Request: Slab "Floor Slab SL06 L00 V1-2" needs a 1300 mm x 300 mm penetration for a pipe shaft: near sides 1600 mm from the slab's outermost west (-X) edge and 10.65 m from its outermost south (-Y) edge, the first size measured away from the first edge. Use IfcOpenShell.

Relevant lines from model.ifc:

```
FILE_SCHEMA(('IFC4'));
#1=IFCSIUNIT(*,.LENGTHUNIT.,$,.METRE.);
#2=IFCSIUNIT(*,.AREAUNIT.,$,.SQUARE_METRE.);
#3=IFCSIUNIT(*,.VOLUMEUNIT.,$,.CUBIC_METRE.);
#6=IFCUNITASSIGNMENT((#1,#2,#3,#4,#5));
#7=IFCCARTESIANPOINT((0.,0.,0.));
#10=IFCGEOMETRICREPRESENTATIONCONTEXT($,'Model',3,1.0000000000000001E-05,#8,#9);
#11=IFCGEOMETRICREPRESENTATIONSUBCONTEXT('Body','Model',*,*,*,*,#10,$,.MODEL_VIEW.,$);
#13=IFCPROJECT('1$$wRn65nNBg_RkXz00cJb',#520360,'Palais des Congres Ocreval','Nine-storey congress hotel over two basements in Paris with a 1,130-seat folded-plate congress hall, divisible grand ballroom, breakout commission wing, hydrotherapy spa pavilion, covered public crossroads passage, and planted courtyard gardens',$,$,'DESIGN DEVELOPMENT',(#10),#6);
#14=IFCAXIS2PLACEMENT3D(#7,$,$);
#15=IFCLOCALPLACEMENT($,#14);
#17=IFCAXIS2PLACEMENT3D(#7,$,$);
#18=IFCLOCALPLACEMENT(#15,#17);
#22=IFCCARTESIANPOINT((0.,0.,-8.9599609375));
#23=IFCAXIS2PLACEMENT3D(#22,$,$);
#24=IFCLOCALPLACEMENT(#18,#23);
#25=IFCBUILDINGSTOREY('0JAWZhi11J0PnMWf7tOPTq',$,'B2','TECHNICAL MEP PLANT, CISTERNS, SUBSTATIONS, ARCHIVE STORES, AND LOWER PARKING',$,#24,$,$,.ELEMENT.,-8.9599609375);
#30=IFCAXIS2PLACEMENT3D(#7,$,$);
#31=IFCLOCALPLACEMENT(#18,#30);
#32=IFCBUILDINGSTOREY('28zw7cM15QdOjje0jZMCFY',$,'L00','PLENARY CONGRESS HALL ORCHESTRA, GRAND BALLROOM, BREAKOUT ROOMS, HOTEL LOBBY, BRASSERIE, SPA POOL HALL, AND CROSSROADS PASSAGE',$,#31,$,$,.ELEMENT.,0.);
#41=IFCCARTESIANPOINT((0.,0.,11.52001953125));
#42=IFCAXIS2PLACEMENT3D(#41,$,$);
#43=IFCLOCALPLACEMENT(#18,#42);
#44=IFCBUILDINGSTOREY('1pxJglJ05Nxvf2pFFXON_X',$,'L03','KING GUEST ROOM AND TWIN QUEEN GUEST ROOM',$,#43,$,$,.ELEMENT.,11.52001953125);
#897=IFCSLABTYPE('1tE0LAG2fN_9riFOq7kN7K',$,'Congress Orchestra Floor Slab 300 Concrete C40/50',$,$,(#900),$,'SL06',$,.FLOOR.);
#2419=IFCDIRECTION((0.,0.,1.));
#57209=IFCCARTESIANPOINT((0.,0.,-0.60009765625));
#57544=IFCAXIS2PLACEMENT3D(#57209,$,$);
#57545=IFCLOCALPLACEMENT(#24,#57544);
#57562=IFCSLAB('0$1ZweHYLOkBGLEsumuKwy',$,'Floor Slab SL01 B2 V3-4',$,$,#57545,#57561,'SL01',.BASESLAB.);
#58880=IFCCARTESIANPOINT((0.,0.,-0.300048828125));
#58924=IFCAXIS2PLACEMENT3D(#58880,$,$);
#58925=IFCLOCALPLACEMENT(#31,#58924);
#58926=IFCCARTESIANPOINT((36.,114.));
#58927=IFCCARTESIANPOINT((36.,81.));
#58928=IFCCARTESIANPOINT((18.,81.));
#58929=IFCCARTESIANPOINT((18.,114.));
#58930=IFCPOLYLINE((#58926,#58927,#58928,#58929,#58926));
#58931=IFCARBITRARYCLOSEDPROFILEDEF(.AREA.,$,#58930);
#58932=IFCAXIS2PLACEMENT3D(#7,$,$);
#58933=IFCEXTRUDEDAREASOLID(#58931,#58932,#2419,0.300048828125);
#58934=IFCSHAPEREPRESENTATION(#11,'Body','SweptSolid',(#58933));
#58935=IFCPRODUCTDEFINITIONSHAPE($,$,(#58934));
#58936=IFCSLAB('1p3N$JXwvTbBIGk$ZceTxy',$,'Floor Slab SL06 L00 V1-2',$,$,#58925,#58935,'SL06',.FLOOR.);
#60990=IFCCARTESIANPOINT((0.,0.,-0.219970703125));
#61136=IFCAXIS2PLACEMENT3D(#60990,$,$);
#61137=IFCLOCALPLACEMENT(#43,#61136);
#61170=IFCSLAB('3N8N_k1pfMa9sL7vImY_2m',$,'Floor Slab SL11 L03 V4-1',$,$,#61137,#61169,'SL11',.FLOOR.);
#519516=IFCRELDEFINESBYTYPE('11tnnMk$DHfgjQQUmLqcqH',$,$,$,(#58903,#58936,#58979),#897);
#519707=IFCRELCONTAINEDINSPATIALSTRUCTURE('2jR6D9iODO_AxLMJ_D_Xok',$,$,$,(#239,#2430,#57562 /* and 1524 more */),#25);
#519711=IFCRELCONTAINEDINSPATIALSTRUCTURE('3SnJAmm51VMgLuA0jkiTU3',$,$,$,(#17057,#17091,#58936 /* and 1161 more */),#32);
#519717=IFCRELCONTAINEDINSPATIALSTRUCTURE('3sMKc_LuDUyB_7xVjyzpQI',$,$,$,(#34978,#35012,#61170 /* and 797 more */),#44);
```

```python
import numpy as np
import ifcopenshell
import ifcopenshell.api.feature
import ifcopenshell.api.geometry
import ifcopenshell.api.root
import ifcopenshell.geom
import ifcopenshell.util.placement
import ifcopenshell.util.representation
import ifcopenshell.util.shape
import ifcopenshell.util.unit

model = ifcopenshell.open("model.ifc")
unit_scale = ifcopenshell.util.unit.calculate_unit_scale(model)
settings = ifcopenshell.geom.settings()


def volume(element):
    """Net volume in cubic metres, openings subtracted."""
    shape = ifcopenshell.geom.create_shape(settings, element)
    return ifcopenshell.util.shape.get_volume(shape.geometry)


slab = model.by_guid("1p3N$JXwvTbBIGk$ZceTxy")
before = volume(slab)

# Extent in the slab's own axes, in metres. The edges named are its -X and -Y sides.
slab_shape = ifcopenshell.geom.create_shape(settings, slab)
vertices = ifcopenshell.util.shape.get_vertices(slab_shape.geometry)
x_min, y_min, bottom = vertices.min(axis=0)
top = vertices[:, 2].max()

opening = ifcopenshell.api.root.create_entity(model, ifc_class="IfcOpeningElement", name="Pipe shaft opening", predefined_type="OPENING")
context = ifcopenshell.util.representation.get_context(model, "Model", "Body", "MODEL_VIEW")
width, depth = 1.3, 0.3
outline = [(0.0, 0.0), (width, 0.0), (width, depth), (0.0, depth), (0.0, 0.0)]
# Overshoot both faces by 50 mm so the cut is clean.
shape = ifcopenshell.api.geometry.add_slab_representation(
    model, context=context, depth=top - bottom + 0.1, polyline=outline
)
ifcopenshell.api.geometry.assign_representation(model, product=opening, representation=shape)

matrix = ifcopenshell.util.placement.get_local_placement(slab.ObjectPlacement)
matrix[:, 3] = matrix @ np.append(np.array([x_min + 1.6, y_min + 10.65, bottom - 0.05]) / unit_scale, 1.0)
ifcopenshell.api.geometry.edit_object_placement(model, product=opening, matrix=matrix, is_si=False)
ifcopenshell.api.feature.add_feature(model, feature=opening, element=slab)

after = volume(slab)

print(f"slab volume {before:.3f} -> {after:.3f} m3")

model.write("model_edited.ifc")
```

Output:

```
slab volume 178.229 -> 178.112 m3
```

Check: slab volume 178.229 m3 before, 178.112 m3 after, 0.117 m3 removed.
